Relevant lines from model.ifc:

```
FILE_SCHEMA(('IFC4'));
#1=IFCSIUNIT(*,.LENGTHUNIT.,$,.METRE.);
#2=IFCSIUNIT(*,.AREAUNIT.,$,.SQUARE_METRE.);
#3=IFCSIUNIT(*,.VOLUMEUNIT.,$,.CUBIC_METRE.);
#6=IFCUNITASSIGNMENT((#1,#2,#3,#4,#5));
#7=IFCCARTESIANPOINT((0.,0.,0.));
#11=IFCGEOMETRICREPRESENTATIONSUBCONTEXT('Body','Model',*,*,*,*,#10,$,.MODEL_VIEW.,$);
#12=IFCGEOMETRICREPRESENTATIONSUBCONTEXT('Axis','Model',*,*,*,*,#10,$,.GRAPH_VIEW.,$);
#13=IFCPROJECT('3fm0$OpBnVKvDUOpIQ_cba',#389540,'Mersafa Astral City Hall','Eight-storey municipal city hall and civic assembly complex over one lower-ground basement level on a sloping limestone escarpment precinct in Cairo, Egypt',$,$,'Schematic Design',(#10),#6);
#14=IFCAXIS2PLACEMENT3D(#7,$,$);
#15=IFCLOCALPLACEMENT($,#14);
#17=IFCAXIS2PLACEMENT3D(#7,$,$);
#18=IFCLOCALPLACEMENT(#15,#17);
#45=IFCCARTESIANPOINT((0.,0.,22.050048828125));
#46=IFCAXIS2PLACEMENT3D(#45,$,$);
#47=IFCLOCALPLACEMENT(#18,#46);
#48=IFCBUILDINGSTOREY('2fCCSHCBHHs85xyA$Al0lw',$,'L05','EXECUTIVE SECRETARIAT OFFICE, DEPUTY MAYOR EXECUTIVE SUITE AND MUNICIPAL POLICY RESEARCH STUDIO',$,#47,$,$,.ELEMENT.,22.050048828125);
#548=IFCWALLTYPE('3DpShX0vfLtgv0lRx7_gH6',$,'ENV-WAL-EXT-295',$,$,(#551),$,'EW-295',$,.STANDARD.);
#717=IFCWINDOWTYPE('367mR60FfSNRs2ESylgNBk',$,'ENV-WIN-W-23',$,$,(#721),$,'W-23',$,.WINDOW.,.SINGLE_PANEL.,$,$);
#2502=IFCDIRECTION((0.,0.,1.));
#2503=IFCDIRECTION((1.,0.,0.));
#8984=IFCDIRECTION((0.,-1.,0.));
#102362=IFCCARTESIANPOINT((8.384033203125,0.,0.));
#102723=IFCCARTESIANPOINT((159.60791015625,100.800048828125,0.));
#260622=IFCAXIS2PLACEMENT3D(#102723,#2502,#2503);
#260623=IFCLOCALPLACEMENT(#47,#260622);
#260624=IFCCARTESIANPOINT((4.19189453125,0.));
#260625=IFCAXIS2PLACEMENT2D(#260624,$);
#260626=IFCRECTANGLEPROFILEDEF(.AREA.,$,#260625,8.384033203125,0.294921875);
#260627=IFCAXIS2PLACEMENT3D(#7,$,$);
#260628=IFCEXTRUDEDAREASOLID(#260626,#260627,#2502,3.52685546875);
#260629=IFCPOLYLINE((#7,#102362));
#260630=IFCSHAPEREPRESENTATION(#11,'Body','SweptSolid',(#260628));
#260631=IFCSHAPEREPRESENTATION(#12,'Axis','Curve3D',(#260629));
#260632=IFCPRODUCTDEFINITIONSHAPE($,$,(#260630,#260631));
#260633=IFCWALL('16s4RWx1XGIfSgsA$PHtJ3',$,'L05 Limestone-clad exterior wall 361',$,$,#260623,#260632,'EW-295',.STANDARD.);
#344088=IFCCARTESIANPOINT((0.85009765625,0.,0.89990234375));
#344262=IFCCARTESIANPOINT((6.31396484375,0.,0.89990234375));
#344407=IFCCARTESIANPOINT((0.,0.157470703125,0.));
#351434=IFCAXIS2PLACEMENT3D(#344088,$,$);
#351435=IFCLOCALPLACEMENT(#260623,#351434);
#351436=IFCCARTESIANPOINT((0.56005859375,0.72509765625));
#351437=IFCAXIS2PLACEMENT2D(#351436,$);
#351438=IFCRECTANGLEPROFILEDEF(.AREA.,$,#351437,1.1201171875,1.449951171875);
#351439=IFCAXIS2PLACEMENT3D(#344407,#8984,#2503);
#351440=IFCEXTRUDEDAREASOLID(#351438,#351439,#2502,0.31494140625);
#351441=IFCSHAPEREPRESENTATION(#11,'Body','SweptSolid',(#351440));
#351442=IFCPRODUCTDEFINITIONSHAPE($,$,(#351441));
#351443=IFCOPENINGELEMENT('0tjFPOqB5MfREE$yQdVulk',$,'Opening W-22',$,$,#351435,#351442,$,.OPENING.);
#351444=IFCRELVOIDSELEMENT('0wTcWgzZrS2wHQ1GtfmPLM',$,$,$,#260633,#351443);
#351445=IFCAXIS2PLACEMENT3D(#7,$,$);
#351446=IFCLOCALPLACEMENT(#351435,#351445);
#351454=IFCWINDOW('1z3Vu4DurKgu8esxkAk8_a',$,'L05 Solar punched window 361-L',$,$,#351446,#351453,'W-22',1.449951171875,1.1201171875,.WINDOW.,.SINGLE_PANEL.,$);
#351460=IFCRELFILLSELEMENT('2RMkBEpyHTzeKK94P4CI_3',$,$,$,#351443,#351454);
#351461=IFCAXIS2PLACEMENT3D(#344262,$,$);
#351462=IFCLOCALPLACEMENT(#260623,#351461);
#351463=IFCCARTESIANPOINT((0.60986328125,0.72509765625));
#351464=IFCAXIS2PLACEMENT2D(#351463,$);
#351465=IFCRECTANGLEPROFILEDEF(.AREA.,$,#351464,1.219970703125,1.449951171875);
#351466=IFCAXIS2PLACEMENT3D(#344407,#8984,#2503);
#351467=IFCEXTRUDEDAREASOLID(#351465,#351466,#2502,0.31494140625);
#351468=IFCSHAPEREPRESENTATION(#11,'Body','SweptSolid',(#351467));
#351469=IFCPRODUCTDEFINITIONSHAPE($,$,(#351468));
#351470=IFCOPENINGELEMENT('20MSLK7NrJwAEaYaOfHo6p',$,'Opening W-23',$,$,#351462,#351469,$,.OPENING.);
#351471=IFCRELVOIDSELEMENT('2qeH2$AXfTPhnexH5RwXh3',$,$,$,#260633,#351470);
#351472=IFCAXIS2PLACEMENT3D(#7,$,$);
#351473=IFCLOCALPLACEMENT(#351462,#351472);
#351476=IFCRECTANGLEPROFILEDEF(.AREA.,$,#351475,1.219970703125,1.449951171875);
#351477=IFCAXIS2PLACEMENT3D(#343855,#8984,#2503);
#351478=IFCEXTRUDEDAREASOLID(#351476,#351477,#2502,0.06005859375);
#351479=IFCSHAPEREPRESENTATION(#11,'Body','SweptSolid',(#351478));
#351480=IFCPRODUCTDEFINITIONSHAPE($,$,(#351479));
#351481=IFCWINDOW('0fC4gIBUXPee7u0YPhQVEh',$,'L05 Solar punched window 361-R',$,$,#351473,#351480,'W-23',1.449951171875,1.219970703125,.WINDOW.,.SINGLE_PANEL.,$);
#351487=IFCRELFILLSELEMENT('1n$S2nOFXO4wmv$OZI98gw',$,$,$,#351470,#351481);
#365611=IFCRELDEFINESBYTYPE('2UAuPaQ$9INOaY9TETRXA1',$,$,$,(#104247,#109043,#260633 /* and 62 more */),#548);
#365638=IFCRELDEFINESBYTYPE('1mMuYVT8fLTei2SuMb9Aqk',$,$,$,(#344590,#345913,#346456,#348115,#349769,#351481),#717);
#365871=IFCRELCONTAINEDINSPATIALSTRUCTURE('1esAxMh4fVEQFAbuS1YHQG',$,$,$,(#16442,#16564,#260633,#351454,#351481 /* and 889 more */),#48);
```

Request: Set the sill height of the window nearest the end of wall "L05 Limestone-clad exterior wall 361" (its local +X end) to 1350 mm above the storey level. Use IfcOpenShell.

```python
import numpy as np
import ifcopenshell
import ifcopenshell.api.geometry
import ifcopenshell.geom
import ifcopenshell.util.element
import ifcopenshell.util.placement
import ifcopenshell.util.shape
import ifcopenshell.util.unit

model = ifcopenshell.open("model.ifc")
unit_scale = ifcopenshell.util.unit.calculate_unit_scale(model)

window = model.by_guid("0fC4gIBUXPee7u0YPhQVEh")
opening = window.FillsVoids[0].RelatingOpeningElement
storey = ifcopenshell.util.element.get_container(window, ifc_class="IfcBuildingStorey")
level = ifcopenshell.util.placement.get_local_placement(storey.ObjectPlacement)[2, 3]

# The opening's origin need not be at the sill, so measure its lowest point.
shape = ifcopenshell.geom.create_shape(ifcopenshell.geom.settings(), opening)
bottom = ifcopenshell.util.shape.get_shape_bottom_elevation(shape, shape.geometry) / unit_scale
dz = level + 1.35 / unit_scale - bottom

shift = np.array([0.0, 0.0, dz])
# The window is placed relative to its opening, so it follows when the opening moves.
matrix = ifcopenshell.util.placement.get_local_placement(opening.ObjectPlacement)
matrix[:3, 3] += shift
ifcopenshell.api.geometry.edit_object_placement(
    model, product=opening, matrix=matrix, is_si=False, should_transform_children=True
)

print(f"moved by {dz * unit_scale:+.3f} m")

model.write("model_updated.ifc")
```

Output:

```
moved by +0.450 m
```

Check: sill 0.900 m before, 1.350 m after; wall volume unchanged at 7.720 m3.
